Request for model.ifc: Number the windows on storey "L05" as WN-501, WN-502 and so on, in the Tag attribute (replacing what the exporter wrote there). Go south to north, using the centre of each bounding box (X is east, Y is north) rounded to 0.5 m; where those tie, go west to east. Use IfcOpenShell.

First a look at what the model holds.

```python
import ifcopenshell
import ifcopenshell.util.element
import ifcopenshell.util.placement

model = ifcopenshell.open("model.ifc")
print(model.schema)
storey = next(s for s in model.by_type("IfcBuildingStorey") if s.Name == "L05")
windows = [e for e in ifcopenshell.util.element.get_decomposition(storey) if e.is_a("IfcWindow")]
for e in sorted(windows, key=lambda e: e.id()):
    origin = ifcopenshell.util.placement.get_local_placement(e.ObjectPlacement)[:3, 3]
    print(e.id(), e.Tag, e.Name, origin.round(2) + 0.0, sep=" | ")
```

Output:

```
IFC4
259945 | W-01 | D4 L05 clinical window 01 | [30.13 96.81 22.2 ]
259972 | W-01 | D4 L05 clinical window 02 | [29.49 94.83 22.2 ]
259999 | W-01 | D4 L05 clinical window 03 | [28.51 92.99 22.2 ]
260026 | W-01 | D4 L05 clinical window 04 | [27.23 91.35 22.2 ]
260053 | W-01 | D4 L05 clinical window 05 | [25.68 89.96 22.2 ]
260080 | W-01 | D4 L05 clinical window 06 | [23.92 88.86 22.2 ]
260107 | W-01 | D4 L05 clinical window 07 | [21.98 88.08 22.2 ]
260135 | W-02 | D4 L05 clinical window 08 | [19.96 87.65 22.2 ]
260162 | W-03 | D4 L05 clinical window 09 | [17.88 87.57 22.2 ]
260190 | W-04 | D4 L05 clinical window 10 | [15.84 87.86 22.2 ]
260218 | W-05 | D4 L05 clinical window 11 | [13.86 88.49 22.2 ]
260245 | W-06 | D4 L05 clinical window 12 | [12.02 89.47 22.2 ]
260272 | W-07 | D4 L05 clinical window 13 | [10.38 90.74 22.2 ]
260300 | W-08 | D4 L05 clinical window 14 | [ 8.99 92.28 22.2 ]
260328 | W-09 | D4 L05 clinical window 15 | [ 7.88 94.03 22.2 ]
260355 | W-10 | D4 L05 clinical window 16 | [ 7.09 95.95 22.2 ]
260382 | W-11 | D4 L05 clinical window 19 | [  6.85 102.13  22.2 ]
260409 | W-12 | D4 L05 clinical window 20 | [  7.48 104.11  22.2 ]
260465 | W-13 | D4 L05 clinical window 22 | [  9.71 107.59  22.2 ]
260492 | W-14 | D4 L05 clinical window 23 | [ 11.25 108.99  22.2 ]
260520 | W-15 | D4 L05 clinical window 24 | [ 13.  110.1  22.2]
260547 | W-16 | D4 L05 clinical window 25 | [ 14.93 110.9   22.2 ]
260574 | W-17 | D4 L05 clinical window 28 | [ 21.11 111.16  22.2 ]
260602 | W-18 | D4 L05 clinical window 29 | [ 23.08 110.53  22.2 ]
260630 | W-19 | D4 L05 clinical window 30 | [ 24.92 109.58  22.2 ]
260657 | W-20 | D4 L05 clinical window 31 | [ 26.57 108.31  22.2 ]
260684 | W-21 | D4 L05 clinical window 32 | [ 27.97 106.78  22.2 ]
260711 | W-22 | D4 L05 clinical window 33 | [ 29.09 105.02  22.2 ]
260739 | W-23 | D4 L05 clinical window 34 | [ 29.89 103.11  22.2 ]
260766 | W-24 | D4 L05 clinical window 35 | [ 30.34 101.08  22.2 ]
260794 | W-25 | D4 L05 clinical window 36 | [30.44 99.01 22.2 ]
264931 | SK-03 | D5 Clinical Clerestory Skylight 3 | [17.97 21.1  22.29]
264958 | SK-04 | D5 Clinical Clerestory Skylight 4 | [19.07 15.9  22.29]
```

```python
import ifcopenshell
import ifcopenshell.geom
import ifcopenshell.util.element
import ifcopenshell.util.shape

model = ifcopenshell.open("model.ifc")
settings = ifcopenshell.geom.settings()
settings.set("use-world-coords", True)


def centre(element):
    shape = ifcopenshell.geom.create_shape(settings, element)
    return ifcopenshell.util.shape.get_bbox_centroid(shape.geometry)


storey = next(s for s in model.by_type("IfcBuildingStorey") if s.Name == "L05")
windows = [e for e in ifcopenshell.util.element.get_decomposition(storey) if e.is_a("IfcWindow")]

# Insertion points can sit at a corner or the storey origin, so sort by the geometry (in metres).
centres = {e: centre(e) for e in windows}
windows.sort(key=lambda e: (round(centres[e][1] / 0.5), centres[e][0]))

for i, e in enumerate(windows, start=1):
    number = f"WN-5{i:02d}"
    e.Tag = number
    print(e.id(), number)

model.write("model_edited.ifc")
```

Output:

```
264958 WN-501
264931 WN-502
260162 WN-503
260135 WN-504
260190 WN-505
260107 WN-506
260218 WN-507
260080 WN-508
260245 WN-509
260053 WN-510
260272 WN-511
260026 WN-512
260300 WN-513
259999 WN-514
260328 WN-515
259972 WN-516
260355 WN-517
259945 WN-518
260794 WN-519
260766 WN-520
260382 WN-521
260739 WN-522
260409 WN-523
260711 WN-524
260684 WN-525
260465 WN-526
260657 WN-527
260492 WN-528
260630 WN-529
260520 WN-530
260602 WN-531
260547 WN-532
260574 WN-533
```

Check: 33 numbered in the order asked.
